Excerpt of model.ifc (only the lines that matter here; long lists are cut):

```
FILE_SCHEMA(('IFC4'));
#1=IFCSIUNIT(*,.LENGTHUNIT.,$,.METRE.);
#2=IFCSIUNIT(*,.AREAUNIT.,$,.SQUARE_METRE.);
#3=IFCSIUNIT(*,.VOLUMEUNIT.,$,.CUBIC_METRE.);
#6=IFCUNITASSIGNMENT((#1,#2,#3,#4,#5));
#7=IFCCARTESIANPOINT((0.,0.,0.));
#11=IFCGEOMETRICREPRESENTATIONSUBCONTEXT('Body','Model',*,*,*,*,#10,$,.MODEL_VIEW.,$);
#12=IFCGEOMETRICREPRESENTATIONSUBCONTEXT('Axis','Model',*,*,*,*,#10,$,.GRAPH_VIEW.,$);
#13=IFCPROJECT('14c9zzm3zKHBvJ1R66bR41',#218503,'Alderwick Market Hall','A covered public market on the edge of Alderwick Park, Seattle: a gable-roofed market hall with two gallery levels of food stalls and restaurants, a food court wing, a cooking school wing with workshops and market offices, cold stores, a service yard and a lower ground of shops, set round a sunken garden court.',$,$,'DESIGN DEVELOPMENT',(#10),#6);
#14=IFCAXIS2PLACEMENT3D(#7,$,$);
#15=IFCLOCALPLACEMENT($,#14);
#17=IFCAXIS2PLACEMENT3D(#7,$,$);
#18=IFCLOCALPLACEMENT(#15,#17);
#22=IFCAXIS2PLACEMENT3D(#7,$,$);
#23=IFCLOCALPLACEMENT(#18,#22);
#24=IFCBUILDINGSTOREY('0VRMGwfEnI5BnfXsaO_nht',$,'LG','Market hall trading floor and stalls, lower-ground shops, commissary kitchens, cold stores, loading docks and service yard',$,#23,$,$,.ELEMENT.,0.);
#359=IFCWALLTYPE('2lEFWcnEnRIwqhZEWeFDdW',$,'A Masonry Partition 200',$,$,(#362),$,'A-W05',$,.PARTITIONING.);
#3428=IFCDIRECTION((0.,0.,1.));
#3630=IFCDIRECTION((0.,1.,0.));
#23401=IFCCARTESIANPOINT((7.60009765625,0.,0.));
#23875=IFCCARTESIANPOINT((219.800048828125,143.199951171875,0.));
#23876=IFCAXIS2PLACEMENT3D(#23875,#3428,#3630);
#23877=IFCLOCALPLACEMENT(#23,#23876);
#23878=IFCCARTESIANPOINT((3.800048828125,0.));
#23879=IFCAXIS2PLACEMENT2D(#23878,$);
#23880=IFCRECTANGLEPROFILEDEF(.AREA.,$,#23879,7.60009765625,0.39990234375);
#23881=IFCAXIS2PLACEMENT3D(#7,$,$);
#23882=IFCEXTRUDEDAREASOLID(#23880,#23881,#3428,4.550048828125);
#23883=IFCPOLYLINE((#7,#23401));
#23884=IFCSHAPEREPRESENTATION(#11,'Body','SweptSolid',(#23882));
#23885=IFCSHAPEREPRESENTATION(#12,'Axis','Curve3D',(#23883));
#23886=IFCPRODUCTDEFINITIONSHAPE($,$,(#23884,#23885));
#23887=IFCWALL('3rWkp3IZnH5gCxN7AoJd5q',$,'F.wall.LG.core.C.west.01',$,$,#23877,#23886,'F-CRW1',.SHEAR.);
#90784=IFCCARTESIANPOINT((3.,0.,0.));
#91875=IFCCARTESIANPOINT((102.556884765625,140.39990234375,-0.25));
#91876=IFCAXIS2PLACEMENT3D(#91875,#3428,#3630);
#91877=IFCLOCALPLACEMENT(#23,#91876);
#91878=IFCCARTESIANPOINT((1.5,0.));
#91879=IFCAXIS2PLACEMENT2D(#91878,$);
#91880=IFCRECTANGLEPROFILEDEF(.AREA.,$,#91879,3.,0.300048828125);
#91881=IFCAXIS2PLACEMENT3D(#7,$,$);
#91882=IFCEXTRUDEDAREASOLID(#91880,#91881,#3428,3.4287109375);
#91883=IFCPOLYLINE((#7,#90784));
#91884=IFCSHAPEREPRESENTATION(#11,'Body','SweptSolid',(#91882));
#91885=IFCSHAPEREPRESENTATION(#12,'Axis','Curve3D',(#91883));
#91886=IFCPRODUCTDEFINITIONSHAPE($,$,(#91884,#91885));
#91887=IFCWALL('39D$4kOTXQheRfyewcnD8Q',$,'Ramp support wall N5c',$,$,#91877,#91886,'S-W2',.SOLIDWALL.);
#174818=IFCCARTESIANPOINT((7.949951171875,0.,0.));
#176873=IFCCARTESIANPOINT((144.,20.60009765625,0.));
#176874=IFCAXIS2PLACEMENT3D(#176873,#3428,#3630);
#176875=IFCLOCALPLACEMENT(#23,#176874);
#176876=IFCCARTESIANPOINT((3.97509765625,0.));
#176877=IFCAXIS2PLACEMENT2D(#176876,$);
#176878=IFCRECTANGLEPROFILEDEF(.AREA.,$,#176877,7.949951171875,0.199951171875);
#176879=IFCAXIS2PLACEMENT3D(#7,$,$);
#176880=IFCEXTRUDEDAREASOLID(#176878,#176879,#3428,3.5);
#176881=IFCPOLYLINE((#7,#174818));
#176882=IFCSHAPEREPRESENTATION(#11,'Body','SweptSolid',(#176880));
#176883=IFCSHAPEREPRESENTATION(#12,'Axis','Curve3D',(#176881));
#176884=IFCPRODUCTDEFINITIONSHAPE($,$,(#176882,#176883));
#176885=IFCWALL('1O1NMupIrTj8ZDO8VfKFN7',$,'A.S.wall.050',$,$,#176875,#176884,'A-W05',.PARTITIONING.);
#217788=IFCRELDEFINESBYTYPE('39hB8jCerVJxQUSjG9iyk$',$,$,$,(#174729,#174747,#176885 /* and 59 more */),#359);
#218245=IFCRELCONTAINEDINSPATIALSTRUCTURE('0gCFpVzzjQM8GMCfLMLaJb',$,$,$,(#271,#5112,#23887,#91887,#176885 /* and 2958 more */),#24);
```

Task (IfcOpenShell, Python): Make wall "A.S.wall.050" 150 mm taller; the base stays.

```python
import ifcopenshell
import ifcopenshell.geom
import ifcopenshell.util.representation
import ifcopenshell.util.shape

model = ifcopenshell.open("model.ifc")
settings = ifcopenshell.geom.settings()


def volume(element):
    """Net volume in cubic metres, openings subtracted."""
    shape = ifcopenshell.geom.create_shape(settings, element)
    return ifcopenshell.util.shape.get_volume(shape.geometry)


wall = model.by_guid("1O1NMupIrTj8ZDO8VfKFN7")
before = volume(wall)

body = ifcopenshell.util.representation.get_representation(wall, "Model", "Body")
solid = body.Items[0]
old_height = solid.Depth
solid.Depth += 0.15
after = volume(wall)

print(f"height {old_height:g} -> {solid.Depth:g}, volume {before:.3f} -> {after:.3f} m3")

model.write("model_v2.ifc")
```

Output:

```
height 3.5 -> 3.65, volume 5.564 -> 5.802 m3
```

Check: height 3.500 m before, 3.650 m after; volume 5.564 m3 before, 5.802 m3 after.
